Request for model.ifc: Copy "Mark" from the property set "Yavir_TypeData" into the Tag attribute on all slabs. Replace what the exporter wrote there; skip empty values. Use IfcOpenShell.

First a look at what the model holds.

```python
import ifcopenshell
import ifcopenshell.util.element

model = ifcopenshell.open("model.ifc")
print(model.schema)
slabs = model.by_type("IfcSlab")
print(len(slabs), "slabs")
for e in slabs[:8]:
    source = ifcopenshell.util.element.get_pset(e, "Yavir_TypeData", "Mark")
    target = e.Tag
    print(e.id(), repr(source), repr(target), sep=" | ")
```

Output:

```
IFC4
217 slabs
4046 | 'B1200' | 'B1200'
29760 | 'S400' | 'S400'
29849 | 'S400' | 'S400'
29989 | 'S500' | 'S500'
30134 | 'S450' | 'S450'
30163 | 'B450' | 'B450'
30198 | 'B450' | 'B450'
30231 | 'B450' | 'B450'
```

```python
import ifcopenshell
import ifcopenshell.util.element

model = ifcopenshell.open("model.ifc")

count = 0
for e in model.by_type("IfcSlab"):
    value = ifcopenshell.util.element.get_pset(e, "Yavir_TypeData", "Mark")
    current = e.Tag
    if not value or not value.strip() or current == value:
        continue
    e.Tag = value
    count += 1

print(count, "slabs updated")

model.write("model_edited.ifc")
```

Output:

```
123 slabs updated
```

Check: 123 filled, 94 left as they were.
